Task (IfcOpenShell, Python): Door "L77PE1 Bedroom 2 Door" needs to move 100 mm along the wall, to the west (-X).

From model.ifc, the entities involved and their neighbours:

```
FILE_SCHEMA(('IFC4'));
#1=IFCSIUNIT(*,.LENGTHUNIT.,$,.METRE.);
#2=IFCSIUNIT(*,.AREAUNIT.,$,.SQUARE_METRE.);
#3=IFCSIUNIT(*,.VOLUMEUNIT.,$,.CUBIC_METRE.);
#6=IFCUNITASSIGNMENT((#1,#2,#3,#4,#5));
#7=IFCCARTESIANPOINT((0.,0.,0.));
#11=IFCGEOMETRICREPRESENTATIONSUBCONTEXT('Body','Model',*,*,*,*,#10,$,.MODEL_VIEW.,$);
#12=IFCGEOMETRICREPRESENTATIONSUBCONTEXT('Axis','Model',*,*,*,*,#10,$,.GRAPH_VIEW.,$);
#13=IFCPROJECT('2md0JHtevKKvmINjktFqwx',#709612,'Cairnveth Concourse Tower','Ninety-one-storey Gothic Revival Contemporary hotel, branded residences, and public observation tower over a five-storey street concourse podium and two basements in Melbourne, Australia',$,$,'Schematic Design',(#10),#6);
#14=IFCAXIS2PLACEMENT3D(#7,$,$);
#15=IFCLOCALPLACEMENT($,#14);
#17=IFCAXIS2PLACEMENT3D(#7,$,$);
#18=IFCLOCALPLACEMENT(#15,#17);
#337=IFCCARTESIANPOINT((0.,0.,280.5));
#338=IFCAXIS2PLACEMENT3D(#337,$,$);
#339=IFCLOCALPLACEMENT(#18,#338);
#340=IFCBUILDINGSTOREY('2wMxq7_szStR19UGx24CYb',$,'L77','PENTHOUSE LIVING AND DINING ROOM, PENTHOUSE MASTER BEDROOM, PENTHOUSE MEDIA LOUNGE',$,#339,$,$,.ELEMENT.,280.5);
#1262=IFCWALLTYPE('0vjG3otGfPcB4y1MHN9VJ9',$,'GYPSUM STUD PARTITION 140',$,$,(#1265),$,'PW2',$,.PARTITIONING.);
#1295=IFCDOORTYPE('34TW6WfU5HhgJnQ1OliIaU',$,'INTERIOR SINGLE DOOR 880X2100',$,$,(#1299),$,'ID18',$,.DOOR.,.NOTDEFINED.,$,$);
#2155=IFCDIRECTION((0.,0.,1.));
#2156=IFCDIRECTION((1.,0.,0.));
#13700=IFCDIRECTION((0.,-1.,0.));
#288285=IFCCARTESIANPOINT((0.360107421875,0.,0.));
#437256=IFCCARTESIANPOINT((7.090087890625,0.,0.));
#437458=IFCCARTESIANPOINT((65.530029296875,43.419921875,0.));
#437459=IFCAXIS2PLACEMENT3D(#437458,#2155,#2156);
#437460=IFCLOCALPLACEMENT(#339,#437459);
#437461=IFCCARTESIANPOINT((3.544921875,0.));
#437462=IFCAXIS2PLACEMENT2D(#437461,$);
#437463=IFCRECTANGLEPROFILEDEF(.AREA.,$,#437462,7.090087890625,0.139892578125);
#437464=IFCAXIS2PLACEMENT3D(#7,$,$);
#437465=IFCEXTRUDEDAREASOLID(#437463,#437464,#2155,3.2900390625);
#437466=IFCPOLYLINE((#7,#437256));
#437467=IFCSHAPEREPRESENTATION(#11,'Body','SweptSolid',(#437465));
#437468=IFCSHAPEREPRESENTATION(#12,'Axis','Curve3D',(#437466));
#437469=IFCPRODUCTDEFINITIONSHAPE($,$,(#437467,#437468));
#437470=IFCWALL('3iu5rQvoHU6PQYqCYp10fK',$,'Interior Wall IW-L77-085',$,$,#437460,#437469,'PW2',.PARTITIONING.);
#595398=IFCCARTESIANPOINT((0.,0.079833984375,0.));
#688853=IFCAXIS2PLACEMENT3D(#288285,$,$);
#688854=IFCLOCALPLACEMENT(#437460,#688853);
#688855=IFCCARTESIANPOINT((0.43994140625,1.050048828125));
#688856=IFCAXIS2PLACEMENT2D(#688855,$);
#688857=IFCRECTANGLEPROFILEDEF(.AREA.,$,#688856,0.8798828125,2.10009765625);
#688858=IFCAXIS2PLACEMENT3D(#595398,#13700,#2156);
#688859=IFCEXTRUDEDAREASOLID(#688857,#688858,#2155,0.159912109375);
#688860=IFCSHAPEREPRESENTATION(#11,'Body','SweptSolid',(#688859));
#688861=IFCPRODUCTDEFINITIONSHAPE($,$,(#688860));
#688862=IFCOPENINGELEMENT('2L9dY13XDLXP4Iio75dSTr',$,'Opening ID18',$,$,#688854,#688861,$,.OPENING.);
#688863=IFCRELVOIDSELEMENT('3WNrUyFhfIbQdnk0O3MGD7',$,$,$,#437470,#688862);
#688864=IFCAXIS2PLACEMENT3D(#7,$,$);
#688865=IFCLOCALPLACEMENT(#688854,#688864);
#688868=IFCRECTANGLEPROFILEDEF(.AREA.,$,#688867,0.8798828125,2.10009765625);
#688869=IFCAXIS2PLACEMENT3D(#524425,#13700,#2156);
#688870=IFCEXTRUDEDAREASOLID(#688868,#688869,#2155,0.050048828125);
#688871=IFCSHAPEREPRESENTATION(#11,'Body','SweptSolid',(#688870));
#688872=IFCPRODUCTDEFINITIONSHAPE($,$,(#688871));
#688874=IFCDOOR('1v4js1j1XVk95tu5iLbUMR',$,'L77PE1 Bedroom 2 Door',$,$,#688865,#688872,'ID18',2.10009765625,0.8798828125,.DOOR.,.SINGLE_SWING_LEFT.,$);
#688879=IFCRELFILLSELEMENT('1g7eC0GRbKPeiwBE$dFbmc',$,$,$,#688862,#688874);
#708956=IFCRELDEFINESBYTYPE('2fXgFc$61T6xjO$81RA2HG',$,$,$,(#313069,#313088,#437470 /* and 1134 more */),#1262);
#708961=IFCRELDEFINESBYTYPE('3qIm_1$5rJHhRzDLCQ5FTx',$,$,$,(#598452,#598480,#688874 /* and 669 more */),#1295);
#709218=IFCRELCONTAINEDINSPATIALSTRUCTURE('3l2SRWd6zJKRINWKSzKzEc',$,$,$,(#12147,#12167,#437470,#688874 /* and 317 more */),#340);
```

```python
import ifcopenshell
import ifcopenshell.api.geometry
import ifcopenshell.util.placement
import ifcopenshell.util.unit

model = ifcopenshell.open("model.ifc")
unit_scale = ifcopenshell.util.unit.calculate_unit_scale(model)

door = model.by_id(688874)
opening = door.FillsVoids[0].RelatingOpeningElement
wall = opening.VoidsElements[0].RelatingBuildingElement

wall_matrix = ifcopenshell.util.placement.get_local_placement(wall.ObjectPlacement)
shift = wall_matrix[:3, 0] * -0.1 / unit_scale
before = ifcopenshell.util.placement.get_local_placement(door.ObjectPlacement)[:3, 3].copy()

# The door is placed relative to its opening, so it follows when the opening moves.
matrix = ifcopenshell.util.placement.get_local_placement(opening.ObjectPlacement)
matrix[:3, 3] += shift
ifcopenshell.api.geometry.edit_object_placement(
    model, product=opening, matrix=matrix, is_si=False, should_transform_children=True
)

after = ifcopenshell.util.placement.get_local_placement(door.ObjectPlacement)[:3, 3]
print("door moved by", (after - before).round(3) + 0.0)

model.write("model_rev.ifc")
```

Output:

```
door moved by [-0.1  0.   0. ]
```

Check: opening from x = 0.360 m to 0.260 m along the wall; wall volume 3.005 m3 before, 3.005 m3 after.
